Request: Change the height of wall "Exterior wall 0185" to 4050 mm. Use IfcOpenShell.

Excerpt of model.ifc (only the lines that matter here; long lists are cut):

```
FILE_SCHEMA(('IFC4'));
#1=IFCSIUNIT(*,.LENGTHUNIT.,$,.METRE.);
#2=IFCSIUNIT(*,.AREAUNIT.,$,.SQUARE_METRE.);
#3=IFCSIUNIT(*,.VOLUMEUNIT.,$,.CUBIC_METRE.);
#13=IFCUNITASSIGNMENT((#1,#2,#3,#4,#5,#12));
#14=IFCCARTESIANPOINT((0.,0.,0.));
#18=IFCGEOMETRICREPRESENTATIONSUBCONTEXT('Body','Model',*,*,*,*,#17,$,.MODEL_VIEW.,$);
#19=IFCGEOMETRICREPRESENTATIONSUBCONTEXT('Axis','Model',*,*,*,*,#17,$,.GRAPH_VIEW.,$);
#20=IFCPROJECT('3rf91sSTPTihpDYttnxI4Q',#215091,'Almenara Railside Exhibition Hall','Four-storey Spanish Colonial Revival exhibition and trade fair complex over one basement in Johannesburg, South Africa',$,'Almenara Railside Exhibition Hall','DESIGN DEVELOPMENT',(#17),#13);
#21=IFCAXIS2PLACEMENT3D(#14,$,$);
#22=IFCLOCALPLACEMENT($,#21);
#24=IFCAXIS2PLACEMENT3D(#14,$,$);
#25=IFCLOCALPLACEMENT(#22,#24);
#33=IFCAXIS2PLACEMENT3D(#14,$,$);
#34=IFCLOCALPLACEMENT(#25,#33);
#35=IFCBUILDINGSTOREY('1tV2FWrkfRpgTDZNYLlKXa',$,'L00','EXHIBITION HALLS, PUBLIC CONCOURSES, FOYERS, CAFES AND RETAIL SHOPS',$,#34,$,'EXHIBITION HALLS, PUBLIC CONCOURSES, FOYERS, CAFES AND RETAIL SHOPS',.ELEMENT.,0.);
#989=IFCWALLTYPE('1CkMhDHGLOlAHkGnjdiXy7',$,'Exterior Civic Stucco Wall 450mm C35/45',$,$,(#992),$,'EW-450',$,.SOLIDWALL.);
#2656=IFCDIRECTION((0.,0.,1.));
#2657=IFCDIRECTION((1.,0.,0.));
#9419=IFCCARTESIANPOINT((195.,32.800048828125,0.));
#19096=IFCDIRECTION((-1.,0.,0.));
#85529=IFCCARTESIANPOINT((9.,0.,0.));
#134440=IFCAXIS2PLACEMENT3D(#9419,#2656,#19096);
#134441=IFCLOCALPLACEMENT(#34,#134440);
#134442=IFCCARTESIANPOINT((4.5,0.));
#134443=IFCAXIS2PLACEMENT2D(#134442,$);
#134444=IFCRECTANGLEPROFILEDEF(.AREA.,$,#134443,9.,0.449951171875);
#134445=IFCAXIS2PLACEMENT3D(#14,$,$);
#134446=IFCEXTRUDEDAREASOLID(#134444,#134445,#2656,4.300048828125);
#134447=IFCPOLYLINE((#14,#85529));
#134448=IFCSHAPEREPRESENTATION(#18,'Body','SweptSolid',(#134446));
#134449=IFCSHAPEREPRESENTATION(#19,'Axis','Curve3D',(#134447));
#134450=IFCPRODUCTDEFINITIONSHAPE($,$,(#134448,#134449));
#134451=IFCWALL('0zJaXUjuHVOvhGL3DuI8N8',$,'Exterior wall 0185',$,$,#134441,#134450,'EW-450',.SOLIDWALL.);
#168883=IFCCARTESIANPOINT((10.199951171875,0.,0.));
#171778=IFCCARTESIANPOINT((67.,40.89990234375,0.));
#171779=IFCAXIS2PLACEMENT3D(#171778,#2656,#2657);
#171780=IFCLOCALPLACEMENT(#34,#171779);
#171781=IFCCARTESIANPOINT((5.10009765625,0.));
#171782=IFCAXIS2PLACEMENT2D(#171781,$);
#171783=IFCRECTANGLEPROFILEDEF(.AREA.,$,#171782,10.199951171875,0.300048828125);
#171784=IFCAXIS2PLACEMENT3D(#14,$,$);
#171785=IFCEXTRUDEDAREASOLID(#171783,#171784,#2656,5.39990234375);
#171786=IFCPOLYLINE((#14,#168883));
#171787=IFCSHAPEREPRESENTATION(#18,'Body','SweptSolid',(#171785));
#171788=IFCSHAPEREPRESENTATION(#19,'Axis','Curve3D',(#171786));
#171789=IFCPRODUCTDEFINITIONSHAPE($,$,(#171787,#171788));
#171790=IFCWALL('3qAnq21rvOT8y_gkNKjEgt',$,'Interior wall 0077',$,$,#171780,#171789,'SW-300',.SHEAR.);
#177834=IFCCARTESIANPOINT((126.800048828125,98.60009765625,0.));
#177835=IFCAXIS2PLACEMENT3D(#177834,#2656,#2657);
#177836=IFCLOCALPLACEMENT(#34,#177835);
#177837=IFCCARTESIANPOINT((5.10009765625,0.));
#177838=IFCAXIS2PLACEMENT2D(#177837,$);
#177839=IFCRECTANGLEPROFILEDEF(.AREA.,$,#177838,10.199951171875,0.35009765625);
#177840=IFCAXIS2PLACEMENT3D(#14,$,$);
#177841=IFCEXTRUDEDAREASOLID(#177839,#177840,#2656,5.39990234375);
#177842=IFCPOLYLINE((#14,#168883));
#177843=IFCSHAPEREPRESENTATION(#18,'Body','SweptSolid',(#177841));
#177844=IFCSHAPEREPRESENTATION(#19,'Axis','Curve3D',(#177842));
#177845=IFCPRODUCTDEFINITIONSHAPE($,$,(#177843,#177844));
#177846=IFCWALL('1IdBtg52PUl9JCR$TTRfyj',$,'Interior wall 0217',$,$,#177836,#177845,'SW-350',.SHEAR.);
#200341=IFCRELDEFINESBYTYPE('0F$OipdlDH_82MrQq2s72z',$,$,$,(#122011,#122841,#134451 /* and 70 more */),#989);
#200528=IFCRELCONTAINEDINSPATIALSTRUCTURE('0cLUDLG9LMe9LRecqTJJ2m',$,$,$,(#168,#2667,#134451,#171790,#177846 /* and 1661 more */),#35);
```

```python
import ifcopenshell
import ifcopenshell.geom
import ifcopenshell.util.representation
import ifcopenshell.util.shape
import ifcopenshell.util.unit

model = ifcopenshell.open("model.ifc")
unit_scale = ifcopenshell.util.unit.calculate_unit_scale(model)
settings = ifcopenshell.geom.settings()


def volume(element):
    """Net volume in cubic metres, openings subtracted."""
    shape = ifcopenshell.geom.create_shape(settings, element)
    return ifcopenshell.util.shape.get_volume(shape.geometry)


wall = model.by_guid("0zJaXUjuHVOvhGL3DuI8N8")
before = volume(wall)

body = ifcopenshell.util.representation.get_representation(wall, "Model", "Body")
solid = body.Items[0]
old_height = solid.Depth
solid.Depth = 4.05 / unit_scale
after = volume(wall)

print(f"height {old_height:g} -> {solid.Depth:g}, volume {before:.3f} -> {after:.3f} m3")

model.write("model_edited.ifc")
```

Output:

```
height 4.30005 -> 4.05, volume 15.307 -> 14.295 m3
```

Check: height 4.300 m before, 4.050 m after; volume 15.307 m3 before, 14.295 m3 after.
